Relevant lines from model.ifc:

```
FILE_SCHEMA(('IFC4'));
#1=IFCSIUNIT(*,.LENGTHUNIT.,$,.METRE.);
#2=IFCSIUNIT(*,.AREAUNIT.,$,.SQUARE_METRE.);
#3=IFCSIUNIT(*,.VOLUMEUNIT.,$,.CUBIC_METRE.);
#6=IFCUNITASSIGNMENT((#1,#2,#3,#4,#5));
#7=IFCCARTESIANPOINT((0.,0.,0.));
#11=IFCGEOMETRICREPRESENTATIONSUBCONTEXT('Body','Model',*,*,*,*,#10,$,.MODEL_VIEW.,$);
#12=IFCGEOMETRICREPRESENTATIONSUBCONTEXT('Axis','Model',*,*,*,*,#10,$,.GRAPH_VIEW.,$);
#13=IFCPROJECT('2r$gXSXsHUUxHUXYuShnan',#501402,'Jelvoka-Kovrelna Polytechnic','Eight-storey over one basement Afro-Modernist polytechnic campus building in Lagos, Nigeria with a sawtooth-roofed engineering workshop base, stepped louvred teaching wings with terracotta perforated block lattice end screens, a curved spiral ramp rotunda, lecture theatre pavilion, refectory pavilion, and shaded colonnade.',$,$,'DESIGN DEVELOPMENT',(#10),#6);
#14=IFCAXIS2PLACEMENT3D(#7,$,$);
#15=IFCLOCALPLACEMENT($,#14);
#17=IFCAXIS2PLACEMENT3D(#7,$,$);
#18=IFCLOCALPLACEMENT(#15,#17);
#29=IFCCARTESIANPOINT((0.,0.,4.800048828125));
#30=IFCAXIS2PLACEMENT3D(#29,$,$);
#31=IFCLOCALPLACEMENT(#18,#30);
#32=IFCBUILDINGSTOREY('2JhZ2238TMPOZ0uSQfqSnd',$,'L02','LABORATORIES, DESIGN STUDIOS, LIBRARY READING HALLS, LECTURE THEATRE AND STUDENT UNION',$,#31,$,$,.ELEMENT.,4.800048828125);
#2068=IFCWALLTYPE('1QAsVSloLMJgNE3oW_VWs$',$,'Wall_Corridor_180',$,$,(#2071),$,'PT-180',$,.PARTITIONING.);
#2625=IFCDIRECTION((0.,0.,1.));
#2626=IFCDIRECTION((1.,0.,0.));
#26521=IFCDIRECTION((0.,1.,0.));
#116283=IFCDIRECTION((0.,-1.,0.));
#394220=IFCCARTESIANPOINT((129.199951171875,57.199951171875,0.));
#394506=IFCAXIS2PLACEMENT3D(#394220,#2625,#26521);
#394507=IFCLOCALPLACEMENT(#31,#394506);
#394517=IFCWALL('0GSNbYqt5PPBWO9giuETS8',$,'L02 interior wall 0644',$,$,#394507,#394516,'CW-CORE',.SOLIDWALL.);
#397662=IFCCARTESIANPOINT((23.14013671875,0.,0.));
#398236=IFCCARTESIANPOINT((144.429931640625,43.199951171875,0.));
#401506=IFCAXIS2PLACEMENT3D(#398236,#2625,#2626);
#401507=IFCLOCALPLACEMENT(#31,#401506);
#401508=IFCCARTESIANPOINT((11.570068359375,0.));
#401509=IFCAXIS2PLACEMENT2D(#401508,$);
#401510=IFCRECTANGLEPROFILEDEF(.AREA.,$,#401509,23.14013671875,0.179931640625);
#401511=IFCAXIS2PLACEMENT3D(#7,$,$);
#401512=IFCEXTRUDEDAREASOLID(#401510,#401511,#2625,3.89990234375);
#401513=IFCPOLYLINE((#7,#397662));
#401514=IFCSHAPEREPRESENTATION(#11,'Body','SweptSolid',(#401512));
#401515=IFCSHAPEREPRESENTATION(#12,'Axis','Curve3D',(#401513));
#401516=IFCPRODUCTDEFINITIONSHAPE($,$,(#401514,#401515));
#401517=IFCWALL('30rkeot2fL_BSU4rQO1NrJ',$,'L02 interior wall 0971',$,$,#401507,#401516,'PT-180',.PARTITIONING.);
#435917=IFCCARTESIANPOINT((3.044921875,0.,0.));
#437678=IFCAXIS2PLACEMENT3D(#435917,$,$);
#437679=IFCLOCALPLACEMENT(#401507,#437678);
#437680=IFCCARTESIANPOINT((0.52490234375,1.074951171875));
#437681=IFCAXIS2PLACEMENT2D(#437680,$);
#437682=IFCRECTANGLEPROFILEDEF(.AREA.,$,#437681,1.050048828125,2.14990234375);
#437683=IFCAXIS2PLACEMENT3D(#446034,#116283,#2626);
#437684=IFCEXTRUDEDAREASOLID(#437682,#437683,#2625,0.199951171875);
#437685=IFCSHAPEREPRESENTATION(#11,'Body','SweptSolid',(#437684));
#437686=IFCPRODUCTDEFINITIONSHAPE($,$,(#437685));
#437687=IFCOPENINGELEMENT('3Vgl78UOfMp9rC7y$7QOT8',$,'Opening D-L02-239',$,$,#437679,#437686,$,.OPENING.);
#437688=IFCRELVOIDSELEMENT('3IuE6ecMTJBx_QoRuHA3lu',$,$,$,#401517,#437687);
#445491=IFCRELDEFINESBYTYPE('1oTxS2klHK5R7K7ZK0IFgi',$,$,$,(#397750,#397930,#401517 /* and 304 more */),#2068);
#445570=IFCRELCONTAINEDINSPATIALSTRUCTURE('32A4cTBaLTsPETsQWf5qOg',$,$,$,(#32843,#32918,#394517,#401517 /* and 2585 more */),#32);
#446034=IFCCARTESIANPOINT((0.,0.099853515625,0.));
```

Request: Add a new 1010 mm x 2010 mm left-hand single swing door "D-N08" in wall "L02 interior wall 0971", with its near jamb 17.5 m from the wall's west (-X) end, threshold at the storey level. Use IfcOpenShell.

```python
import numpy as np
import ifcopenshell
import ifcopenshell.api.feature
import ifcopenshell.api.geometry
import ifcopenshell.api.root
import ifcopenshell.api.spatial
import ifcopenshell.geom
import ifcopenshell.util.element
import ifcopenshell.util.placement
import ifcopenshell.util.representation
import ifcopenshell.util.shape
import ifcopenshell.util.unit

model = ifcopenshell.open("model.ifc")
unit_scale = ifcopenshell.util.unit.calculate_unit_scale(model)
settings = ifcopenshell.geom.settings()


def volume(element):
    """Net volume in cubic metres, openings subtracted."""
    shape = ifcopenshell.geom.create_shape(settings, element)
    return ifcopenshell.util.shape.get_volume(shape.geometry)


wall = model.by_guid("30rkeot2fL_BSU4rQO1NrJ")
storey = ifcopenshell.util.element.get_container(wall, ifc_class="IfcBuildingStorey")
context = ifcopenshell.util.representation.get_context(model, "Model", "Body", "MODEL_VIEW")
before = volume(wall)

width, height, from_end, sill = 1.01, 2.01, 17.5, 0.0  # metres

# The wall runs along its own X axis, and the end named is its -X end.
wall_shape = ifcopenshell.geom.create_shape(settings, wall)
x, y, z = ifcopenshell.util.shape.get_vertices(wall_shape.geometry).T
start = x.min() + from_end
face, thickness = float(y.min()), float(y.max() - y.min())
wall_matrix = ifcopenshell.util.placement.get_local_placement(wall.ObjectPlacement)
level = ifcopenshell.util.placement.get_local_placement(storey.ObjectPlacement)[2, 3]


def in_wall(x, y):
    """Placement at x, y metres in the wall's axes, at sill height."""
    matrix = wall_matrix.copy()
    matrix[:, 3] = wall_matrix @ np.array([x / unit_scale, y / unit_scale, 0.0, 1.0])
    matrix[2, 3] = level + sill / unit_scale
    return matrix


# Opening: a box that overshoots both wall faces by 50 mm.
opening = ifcopenshell.api.root.create_entity(model, ifc_class="IfcOpeningElement", predefined_type="OPENING")
box = ifcopenshell.api.geometry.add_wall_representation(
    model, context=context, length=width, height=height, thickness=thickness + 0.1
)
ifcopenshell.api.geometry.assign_representation(model, product=opening, representation=box)
ifcopenshell.api.geometry.edit_object_placement(model, product=opening, matrix=in_wall(start, face - 0.05), is_si=False)
ifcopenshell.api.feature.add_feature(model, feature=opening, element=wall)

door = ifcopenshell.api.root.create_entity(model, ifc_class="IfcDoor", name="D-N08", predefined_type="DOOR")
door.OverallWidth, door.OverallHeight = width / unit_scale, height / unit_scale
door.OperationType = "SINGLE_SWING_LEFT"
body = ifcopenshell.api.geometry.add_door_representation(
    model,
    context=context,
    overall_width=door.OverallWidth,
    overall_height=door.OverallHeight,
    operation_type="SINGLE_SWING_LEFT",
    lining_properties={"LiningDepth": thickness / unit_scale, "ThresholdDepth": thickness / unit_scale},
)
ifcopenshell.api.geometry.assign_representation(model, product=door, representation=body)
ifcopenshell.api.spatial.assign_container(model, products=[door], relating_structure=storey)
ifcopenshell.api.feature.add_filling(model, opening=opening, element=door)

# The lining spans the wall, so the door starts at the wall face.
ifcopenshell.api.geometry.edit_object_placement(model, product=door, matrix=in_wall(start, face), is_si=False)

after = volume(wall)

print(f"wall volume {before:.3f} -> {after:.3f} m3")

model.write("model_updated.ifc")
```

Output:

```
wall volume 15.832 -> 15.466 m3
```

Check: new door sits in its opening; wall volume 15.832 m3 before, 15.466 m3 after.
